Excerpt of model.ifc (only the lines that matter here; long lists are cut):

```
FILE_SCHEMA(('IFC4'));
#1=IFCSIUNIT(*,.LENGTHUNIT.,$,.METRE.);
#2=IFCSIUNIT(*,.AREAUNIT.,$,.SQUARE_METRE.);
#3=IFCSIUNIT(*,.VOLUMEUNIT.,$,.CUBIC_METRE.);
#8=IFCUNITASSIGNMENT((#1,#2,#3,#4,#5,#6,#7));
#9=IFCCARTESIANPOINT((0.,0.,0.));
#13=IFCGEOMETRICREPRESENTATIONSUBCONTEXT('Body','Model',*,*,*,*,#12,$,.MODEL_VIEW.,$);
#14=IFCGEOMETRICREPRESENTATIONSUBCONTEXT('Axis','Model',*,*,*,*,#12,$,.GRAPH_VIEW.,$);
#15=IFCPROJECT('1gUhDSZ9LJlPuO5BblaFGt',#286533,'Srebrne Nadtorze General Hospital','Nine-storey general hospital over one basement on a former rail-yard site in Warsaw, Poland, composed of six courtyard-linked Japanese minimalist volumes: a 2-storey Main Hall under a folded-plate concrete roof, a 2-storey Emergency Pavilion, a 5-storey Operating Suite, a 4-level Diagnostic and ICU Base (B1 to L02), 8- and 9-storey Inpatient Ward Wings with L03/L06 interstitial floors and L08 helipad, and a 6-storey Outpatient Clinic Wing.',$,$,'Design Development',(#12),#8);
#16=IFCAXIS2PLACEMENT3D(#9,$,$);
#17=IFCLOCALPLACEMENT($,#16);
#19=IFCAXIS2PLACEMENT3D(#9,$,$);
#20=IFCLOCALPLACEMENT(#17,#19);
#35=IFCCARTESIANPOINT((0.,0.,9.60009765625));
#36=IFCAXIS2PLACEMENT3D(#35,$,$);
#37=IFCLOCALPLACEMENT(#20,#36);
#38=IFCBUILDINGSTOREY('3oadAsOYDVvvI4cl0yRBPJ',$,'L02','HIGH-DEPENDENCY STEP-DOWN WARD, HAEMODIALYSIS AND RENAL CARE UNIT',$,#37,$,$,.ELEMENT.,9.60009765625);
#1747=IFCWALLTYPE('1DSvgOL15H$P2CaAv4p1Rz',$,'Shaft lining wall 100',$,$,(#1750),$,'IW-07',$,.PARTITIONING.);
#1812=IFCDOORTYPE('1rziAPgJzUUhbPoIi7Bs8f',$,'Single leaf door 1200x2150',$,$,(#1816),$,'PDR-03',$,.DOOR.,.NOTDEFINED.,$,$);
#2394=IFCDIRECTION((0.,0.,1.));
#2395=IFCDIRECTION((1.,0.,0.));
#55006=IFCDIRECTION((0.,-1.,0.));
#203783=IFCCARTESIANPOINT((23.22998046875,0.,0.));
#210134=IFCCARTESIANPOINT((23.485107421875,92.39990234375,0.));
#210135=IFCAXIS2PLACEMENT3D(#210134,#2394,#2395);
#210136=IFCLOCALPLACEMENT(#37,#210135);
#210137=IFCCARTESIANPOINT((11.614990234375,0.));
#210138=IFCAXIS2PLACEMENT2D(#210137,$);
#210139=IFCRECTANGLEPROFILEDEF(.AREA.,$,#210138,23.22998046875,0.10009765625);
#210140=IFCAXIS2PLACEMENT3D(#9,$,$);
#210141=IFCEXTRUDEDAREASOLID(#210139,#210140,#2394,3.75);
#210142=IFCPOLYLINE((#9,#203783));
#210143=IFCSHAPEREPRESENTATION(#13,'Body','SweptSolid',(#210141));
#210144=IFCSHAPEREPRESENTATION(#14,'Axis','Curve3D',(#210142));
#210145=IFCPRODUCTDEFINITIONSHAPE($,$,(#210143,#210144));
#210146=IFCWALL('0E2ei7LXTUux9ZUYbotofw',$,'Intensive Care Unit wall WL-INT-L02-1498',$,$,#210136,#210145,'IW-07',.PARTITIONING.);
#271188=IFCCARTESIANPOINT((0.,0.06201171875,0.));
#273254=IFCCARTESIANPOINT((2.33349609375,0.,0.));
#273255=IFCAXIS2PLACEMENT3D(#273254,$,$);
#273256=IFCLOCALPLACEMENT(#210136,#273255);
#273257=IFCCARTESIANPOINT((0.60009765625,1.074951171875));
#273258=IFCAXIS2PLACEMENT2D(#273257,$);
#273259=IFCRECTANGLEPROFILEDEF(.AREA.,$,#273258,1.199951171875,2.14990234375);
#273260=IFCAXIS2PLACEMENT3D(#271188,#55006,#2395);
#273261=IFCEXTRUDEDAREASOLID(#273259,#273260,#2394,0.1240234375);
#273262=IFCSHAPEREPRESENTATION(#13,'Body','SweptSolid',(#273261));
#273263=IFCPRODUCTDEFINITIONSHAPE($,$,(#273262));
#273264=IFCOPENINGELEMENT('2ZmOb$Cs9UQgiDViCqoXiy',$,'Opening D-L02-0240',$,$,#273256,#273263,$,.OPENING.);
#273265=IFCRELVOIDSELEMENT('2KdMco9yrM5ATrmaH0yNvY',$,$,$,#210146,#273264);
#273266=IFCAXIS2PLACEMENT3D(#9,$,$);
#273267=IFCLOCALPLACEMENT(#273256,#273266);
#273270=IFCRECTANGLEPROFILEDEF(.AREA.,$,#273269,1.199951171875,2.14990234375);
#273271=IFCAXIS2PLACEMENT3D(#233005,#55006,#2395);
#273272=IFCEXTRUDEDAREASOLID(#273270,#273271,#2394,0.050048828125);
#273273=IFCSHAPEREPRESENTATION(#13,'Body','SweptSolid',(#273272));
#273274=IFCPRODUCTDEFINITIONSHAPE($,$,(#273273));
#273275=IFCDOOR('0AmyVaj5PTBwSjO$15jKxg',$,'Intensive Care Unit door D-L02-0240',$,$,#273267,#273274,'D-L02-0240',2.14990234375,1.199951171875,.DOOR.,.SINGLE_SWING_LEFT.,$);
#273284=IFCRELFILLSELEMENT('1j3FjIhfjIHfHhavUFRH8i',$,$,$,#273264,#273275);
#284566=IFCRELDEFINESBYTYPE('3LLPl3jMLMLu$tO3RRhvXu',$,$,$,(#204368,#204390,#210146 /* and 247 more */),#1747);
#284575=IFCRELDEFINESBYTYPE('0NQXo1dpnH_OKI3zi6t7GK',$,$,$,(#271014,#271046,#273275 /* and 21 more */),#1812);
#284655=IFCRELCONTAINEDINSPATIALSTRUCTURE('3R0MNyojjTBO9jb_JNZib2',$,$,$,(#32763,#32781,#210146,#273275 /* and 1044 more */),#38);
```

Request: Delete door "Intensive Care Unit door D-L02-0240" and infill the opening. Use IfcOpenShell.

```python
import ifcopenshell
import ifcopenshell.api.feature
import ifcopenshell.api.root
import ifcopenshell.geom
import ifcopenshell.util.shape

model = ifcopenshell.open("model.ifc")
settings = ifcopenshell.geom.settings()


def volume(element):
    """Net volume in cubic metres, openings subtracted."""
    shape = ifcopenshell.geom.create_shape(settings, element)
    return ifcopenshell.util.shape.get_volume(shape.geometry)


door = model.by_id(273275)
opening = door.FillsVoids[0].RelatingOpeningElement
wall = opening.VoidsElements[0].RelatingBuildingElement
before = volume(wall)

ifcopenshell.api.root.remove_product(model, product=door)
ifcopenshell.api.feature.remove_feature(model, feature=opening)

after = volume(wall)

print(f"wall volume {before:.3f} -> {after:.3f} m3")

model.write("model_updated.ifc")
```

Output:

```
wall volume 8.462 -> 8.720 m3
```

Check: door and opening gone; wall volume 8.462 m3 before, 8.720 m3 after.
